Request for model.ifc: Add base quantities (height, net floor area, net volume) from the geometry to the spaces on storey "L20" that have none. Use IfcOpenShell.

First a look at what the model holds.

```python
import ifcopenshell
import ifcopenshell.util.element
import ifcopenshell.util.unit

model = ifcopenshell.open("model.ifc")
print(model.schema)
for unit_type in ("LENGTHUNIT", "AREAUNIT", "VOLUMEUNIT"):
    print(unit_type, ifcopenshell.util.unit.calculate_unit_scale(model, unit_type))
storey = next(s for s in model.by_type("IfcBuildingStorey") if s.Name == "L20")
spaces = [e for e in ifcopenshell.util.element.get_decomposition(storey) if e.is_a("IfcSpace")]
for e in sorted(spaces, key=lambda e: e.id()):
    print(e.id(), e.is_a(), e.Name, list(ifcopenshell.util.element.get_psets(e, qtos_only=True)), sep=" | ")
```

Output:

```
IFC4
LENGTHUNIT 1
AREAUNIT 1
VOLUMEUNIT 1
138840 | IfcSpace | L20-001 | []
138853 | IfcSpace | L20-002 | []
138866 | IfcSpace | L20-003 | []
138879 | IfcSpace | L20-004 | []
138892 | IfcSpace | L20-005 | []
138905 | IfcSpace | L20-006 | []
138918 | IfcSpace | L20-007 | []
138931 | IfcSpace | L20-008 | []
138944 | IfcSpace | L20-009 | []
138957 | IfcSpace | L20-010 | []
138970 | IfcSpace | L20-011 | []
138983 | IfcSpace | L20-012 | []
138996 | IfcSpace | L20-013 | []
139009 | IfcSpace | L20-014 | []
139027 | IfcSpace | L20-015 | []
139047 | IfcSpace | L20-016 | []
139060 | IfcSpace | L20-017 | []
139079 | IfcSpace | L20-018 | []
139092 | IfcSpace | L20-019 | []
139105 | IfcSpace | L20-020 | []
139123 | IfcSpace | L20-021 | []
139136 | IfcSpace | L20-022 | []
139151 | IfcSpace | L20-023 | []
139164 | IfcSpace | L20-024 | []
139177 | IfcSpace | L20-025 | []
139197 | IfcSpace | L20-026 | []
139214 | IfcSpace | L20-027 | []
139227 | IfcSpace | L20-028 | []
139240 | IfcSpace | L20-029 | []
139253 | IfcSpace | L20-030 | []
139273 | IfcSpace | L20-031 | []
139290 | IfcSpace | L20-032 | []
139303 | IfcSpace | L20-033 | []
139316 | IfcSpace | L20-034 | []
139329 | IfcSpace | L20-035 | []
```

```python
import ifcopenshell
import ifcopenshell.api.pset
import ifcopenshell.geom
import ifcopenshell.util.element
import ifcopenshell.util.shape
import ifcopenshell.util.unit

model = ifcopenshell.open("model.ifc")
unit_scale = ifcopenshell.util.unit.calculate_unit_scale(model)
area_scale = ifcopenshell.util.unit.calculate_unit_scale(model, "AREAUNIT")
volume_scale = ifcopenshell.util.unit.calculate_unit_scale(model, "VOLUMEUNIT")
settings = ifcopenshell.geom.settings()

storey = next(s for s in model.by_type("IfcBuildingStorey") if s.Name == "L20")
spaces = [e for e in ifcopenshell.util.element.get_decomposition(storey) if e.is_a("IfcSpace")]

for e in sorted(spaces, key=lambda e: e.id()):
    if ifcopenshell.util.element.get_psets(e, qtos_only=True, should_inherit=False):
        continue
    # Geometry comes back in metres, in the element's own axes.
    shape = ifcopenshell.geom.create_shape(settings, e)
    values = {
        "Height": ifcopenshell.util.shape.get_z(shape.geometry) / unit_scale,
        "NetFloorArea": ifcopenshell.util.shape.get_footprint_area(shape.geometry) / area_scale,
        "NetVolume": ifcopenshell.util.shape.get_volume(shape.geometry) / volume_scale,
    }
    qto = ifcopenshell.api.pset.add_qto(model, product=e, name="Qto_SpaceBaseQuantities")
    ifcopenshell.api.pset.edit_qto(model, qto=qto, properties=values)
    print(e.id(), {k: round(v, 3) for k, v in values.items()})

model.write("model_v2.ifc")
```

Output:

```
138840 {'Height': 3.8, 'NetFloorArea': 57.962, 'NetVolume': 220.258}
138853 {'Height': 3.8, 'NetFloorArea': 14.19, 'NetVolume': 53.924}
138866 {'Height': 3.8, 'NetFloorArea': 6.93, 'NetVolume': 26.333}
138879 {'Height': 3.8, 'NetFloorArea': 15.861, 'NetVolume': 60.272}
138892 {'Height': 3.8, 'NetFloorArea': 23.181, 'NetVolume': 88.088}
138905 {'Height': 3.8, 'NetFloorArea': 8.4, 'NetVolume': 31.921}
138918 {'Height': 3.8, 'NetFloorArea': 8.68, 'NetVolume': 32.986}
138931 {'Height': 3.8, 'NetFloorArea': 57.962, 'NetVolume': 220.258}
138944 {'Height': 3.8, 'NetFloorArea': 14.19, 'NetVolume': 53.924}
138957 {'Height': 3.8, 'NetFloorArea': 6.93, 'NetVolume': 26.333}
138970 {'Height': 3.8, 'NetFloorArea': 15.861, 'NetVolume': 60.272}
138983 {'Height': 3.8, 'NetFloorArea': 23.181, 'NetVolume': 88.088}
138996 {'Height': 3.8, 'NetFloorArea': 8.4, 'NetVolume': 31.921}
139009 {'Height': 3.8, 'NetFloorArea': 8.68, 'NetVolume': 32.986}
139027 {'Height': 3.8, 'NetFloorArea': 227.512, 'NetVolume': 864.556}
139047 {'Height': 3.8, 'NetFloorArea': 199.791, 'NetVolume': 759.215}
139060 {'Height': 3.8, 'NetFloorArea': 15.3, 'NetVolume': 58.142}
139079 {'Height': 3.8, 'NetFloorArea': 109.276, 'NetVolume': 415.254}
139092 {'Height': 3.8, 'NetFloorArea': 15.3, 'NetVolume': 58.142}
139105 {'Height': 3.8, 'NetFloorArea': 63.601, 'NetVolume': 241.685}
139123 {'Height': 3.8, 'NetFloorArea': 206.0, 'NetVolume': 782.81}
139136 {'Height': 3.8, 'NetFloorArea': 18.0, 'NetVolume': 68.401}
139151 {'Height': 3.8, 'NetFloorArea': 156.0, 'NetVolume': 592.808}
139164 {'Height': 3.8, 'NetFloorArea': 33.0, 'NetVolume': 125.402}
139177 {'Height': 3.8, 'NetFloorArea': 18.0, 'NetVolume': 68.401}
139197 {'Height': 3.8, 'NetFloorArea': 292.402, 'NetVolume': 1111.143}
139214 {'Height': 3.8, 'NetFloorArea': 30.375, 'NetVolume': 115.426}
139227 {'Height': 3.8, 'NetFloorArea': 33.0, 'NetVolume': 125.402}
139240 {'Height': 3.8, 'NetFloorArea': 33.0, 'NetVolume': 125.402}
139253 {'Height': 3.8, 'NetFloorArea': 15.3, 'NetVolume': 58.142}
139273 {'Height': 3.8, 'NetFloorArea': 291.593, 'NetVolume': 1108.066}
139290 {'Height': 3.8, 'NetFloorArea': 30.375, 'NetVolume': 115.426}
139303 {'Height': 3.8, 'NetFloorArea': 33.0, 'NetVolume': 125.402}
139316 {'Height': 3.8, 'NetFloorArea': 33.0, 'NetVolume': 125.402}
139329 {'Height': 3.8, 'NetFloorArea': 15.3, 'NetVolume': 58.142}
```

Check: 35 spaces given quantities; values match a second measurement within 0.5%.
